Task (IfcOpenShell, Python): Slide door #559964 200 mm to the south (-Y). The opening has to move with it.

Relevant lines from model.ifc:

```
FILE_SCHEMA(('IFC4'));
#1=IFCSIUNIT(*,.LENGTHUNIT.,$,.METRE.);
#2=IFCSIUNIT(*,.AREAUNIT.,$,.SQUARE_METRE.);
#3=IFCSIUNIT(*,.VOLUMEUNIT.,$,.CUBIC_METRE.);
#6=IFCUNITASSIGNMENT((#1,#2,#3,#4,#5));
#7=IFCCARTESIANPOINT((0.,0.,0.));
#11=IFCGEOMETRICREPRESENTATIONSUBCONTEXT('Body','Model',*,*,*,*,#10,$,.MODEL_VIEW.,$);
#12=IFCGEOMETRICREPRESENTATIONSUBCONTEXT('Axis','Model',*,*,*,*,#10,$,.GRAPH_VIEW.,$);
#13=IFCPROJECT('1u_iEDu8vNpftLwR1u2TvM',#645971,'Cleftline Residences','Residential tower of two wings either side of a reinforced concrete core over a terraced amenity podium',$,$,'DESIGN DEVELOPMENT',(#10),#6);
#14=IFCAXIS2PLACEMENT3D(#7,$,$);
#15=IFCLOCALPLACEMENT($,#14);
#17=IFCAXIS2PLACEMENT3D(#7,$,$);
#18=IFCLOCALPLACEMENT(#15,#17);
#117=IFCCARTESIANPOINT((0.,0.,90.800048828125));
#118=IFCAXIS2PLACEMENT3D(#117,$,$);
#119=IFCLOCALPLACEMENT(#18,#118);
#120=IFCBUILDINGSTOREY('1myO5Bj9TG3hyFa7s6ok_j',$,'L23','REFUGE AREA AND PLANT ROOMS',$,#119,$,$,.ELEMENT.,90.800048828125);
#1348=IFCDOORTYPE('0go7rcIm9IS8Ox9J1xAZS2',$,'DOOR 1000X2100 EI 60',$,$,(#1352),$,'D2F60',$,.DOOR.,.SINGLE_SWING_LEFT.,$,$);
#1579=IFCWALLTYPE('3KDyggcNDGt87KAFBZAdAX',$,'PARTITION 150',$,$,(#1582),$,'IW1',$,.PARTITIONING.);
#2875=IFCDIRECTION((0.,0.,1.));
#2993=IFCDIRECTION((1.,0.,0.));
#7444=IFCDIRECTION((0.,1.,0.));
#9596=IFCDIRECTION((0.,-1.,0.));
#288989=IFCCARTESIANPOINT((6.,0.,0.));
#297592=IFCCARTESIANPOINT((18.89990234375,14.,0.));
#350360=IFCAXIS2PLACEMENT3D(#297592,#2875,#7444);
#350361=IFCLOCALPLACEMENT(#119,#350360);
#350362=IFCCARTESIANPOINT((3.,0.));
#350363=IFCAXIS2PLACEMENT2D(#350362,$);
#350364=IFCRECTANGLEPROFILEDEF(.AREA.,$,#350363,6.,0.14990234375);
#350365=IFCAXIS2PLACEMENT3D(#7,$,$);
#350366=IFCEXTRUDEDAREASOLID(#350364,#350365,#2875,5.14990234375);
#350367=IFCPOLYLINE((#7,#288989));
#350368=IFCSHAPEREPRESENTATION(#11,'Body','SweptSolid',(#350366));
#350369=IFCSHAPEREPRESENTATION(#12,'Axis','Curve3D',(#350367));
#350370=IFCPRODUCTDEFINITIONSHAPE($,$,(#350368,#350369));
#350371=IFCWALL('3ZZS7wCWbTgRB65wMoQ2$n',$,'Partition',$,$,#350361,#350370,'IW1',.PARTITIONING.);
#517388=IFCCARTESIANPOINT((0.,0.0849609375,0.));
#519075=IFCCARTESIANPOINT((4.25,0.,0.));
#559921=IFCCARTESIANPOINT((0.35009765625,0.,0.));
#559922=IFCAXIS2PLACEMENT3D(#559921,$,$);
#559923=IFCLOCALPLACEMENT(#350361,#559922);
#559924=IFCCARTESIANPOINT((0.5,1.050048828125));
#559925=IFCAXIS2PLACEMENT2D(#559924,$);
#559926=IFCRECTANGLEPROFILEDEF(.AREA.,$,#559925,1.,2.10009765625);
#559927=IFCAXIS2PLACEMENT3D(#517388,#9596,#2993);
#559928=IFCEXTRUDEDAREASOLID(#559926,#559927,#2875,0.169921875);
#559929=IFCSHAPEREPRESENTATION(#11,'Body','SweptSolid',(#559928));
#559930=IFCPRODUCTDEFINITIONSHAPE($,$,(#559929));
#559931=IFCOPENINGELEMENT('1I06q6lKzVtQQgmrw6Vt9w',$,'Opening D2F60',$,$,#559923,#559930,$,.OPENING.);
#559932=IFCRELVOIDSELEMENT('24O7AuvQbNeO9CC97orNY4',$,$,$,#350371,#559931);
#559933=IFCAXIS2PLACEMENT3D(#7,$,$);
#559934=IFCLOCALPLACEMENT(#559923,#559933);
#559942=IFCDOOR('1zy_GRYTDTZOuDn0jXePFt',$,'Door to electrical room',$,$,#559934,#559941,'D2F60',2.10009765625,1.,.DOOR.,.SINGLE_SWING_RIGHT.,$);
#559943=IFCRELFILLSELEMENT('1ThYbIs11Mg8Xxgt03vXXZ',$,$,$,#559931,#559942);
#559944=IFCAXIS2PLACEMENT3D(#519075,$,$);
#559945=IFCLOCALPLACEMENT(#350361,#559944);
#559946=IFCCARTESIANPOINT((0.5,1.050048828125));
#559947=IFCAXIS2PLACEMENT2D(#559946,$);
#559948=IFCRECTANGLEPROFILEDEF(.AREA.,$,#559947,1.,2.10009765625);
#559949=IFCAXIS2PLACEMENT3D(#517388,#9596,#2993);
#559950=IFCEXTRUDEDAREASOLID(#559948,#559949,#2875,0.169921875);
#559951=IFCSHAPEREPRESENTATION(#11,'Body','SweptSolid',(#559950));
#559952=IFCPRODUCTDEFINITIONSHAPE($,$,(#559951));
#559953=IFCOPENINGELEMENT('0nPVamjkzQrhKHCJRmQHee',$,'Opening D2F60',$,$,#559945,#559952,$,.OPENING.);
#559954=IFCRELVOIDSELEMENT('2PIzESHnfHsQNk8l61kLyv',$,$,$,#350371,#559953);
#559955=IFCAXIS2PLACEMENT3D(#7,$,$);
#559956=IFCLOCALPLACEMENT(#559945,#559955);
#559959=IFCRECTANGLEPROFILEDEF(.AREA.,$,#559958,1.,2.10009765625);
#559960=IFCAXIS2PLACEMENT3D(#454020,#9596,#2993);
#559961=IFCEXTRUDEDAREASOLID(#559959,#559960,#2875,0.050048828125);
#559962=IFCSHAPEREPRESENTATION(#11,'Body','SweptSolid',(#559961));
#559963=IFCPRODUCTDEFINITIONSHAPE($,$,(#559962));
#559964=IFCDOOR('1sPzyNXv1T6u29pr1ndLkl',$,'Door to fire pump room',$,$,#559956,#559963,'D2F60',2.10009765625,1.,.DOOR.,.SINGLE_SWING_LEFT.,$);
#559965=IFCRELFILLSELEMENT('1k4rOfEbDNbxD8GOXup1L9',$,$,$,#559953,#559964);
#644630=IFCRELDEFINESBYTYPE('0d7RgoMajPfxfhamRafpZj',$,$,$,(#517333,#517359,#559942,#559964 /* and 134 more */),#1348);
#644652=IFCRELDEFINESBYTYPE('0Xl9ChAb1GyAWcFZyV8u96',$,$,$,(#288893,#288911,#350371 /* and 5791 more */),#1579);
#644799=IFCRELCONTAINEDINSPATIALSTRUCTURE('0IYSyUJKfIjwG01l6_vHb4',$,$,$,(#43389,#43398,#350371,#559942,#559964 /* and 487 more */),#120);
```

```python
import ifcopenshell
import ifcopenshell.api.geometry
import ifcopenshell.util.placement
import ifcopenshell.util.unit

model = ifcopenshell.open("model.ifc")
unit_scale = ifcopenshell.util.unit.calculate_unit_scale(model)

door = model.by_guid("1sPzyNXv1T6u29pr1ndLkl")
opening = door.FillsVoids[0].RelatingOpeningElement
wall = opening.VoidsElements[0].RelatingBuildingElement

wall_matrix = ifcopenshell.util.placement.get_local_placement(wall.ObjectPlacement)
shift = wall_matrix[:3, 0] * -0.2 / unit_scale
before = ifcopenshell.util.placement.get_local_placement(door.ObjectPlacement)[:3, 3].copy()

# The door is placed relative to its opening, so it follows when the opening moves.
matrix = ifcopenshell.util.placement.get_local_placement(opening.ObjectPlacement)
matrix[:3, 3] += shift
ifcopenshell.api.geometry.edit_object_placement(
    model, product=opening, matrix=matrix, is_si=False, should_transform_children=True
)

after = ifcopenshell.util.placement.get_local_placement(door.ObjectPlacement)[:3, 3]
print("door moved by", (after - before).round(3) + 0.0)

model.write("model_rev.ifc")
```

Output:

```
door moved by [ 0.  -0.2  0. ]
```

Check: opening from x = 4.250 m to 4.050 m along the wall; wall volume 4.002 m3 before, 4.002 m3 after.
